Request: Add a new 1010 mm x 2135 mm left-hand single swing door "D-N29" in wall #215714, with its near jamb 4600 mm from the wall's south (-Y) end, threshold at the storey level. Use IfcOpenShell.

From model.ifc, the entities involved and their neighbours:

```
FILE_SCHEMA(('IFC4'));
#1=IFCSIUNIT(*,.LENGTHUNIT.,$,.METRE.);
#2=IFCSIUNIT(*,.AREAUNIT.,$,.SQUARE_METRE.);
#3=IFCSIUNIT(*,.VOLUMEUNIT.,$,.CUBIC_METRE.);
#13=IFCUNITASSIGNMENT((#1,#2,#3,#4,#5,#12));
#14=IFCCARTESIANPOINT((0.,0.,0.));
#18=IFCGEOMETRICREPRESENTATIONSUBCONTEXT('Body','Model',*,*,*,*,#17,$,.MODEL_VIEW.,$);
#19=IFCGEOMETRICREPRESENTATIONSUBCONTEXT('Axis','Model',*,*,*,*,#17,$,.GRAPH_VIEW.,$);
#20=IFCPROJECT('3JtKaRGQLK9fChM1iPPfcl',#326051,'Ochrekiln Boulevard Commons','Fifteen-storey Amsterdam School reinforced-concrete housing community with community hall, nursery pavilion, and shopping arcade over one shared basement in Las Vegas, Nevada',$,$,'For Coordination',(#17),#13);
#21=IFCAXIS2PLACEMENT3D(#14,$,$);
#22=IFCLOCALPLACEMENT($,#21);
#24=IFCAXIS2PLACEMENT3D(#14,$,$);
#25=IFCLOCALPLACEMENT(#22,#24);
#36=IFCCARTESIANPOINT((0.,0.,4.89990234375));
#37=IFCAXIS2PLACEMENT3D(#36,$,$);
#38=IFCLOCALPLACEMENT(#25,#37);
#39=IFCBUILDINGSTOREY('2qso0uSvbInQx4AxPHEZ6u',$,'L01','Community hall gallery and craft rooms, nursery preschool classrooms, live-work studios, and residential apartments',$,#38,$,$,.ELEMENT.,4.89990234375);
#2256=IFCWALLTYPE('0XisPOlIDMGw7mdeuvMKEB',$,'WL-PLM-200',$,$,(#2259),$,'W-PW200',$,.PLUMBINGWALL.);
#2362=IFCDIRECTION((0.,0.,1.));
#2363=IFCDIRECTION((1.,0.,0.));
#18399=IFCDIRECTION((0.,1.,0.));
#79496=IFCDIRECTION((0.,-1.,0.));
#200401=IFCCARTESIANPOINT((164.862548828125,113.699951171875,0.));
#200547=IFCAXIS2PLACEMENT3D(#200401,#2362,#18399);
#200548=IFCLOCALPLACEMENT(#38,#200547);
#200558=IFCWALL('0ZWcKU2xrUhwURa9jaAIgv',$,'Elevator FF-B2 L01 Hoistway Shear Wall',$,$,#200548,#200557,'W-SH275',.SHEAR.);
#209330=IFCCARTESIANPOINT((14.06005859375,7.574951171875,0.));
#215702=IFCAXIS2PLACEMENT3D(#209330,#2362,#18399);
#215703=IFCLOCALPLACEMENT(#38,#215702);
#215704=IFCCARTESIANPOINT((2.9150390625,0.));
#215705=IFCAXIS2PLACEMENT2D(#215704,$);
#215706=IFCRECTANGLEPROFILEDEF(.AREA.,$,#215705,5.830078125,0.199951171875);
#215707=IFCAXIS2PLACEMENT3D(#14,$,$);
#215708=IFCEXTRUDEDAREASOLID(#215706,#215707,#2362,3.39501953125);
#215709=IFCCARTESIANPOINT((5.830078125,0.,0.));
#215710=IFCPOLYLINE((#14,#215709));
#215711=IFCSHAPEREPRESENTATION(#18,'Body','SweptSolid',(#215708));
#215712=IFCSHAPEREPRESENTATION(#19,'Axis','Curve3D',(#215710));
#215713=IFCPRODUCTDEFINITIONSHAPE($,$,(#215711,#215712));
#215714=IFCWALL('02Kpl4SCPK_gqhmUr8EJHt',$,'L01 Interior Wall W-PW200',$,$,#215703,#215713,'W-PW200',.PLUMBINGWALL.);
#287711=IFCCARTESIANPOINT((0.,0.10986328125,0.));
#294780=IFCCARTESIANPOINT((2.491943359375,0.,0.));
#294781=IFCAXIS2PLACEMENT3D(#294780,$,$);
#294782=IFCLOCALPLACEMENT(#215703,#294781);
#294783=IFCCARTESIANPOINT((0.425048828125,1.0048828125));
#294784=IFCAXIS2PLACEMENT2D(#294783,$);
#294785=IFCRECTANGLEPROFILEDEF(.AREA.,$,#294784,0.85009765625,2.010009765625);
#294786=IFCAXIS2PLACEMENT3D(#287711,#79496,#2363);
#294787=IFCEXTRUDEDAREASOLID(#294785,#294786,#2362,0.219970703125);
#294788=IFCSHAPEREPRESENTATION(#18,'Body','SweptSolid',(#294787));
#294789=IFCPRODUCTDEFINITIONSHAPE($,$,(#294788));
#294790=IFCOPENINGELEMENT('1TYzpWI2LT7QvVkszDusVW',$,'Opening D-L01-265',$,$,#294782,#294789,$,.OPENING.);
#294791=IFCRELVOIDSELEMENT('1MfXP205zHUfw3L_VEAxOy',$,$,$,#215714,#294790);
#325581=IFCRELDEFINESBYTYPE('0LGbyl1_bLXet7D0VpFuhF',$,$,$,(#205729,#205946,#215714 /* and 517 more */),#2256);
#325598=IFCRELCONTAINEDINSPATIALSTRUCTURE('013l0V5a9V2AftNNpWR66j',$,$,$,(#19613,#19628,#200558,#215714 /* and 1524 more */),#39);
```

```python
import numpy as np
import ifcopenshell
import ifcopenshell.api.feature
import ifcopenshell.api.geometry
import ifcopenshell.api.root
import ifcopenshell.api.spatial
import ifcopenshell.geom
import ifcopenshell.util.element
import ifcopenshell.util.placement
import ifcopenshell.util.representation
import ifcopenshell.util.shape
import ifcopenshell.util.unit

model = ifcopenshell.open("model.ifc")
unit_scale = ifcopenshell.util.unit.calculate_unit_scale(model)
settings = ifcopenshell.geom.settings()


def volume(element):
    """Net volume in cubic metres, openings subtracted."""
    shape = ifcopenshell.geom.create_shape(settings, element)
    return ifcopenshell.util.shape.get_volume(shape.geometry)


wall = model.by_guid("02Kpl4SCPK_gqhmUr8EJHt")
storey = ifcopenshell.util.element.get_container(wall, ifc_class="IfcBuildingStorey")
context = ifcopenshell.util.representation.get_context(model, "Model", "Body", "MODEL_VIEW")
before = volume(wall)

width, height, from_end, sill = 1.01, 2.135, 4.6, 0.0  # metres

# The wall runs along its own X axis, and the end named is its -X end.
wall_shape = ifcopenshell.geom.create_shape(settings, wall)
x, y, z = ifcopenshell.util.shape.get_vertices(wall_shape.geometry).T
start = x.min() + from_end
face, thickness = float(y.min()), float(y.max() - y.min())
wall_matrix = ifcopenshell.util.placement.get_local_placement(wall.ObjectPlacement)
level = ifcopenshell.util.placement.get_local_placement(storey.ObjectPlacement)[2, 3]


def in_wall(x, y):
    """Placement at x, y metres in the wall's axes, at sill height."""
    matrix = wall_matrix.copy()
    matrix[:, 3] = wall_matrix @ np.array([x / unit_scale, y / unit_scale, 0.0, 1.0])
    matrix[2, 3] = level + sill / unit_scale
    return matrix


# Opening: a box that overshoots both wall faces by 50 mm.
opening = ifcopenshell.api.root.create_entity(model, ifc_class="IfcOpeningElement", predefined_type="OPENING")
box = ifcopenshell.api.geometry.add_wall_representation(
    model, context=context, length=width, height=height, thickness=thickness + 0.1
)
ifcopenshell.api.geometry.assign_representation(model, product=opening, representation=box)
ifcopenshell.api.geometry.edit_object_placement(model, product=opening, matrix=in_wall(start, face - 0.05), is_si=False)
ifcopenshell.api.feature.add_feature(model, feature=opening, element=wall)

door = ifcopenshell.api.root.create_entity(model, ifc_class="IfcDoor", name="D-N29", predefined_type="DOOR")
door.OverallWidth, door.OverallHeight = width / unit_scale, height / unit_scale
door.OperationType = "SINGLE_SWING_LEFT"
body = ifcopenshell.api.geometry.add_door_representation(
    model,
    context=context,
    overall_width=door.OverallWidth,
    overall_height=door.OverallHeight,
    operation_type="SINGLE_SWING_LEFT",
    lining_properties={"LiningDepth": thickness / unit_scale, "ThresholdDepth": thickness / unit_scale},
)
ifcopenshell.api.geometry.assign_representation(model, product=door, representation=body)
ifcopenshell.api.spatial.assign_container(model, products=[door], relating_structure=storey)
ifcopenshell.api.feature.add_filling(model, opening=opening, element=door)

# The lining spans the wall, so the door starts at the wall face.
ifcopenshell.api.geometry.edit_object_placement(model, product=door, matrix=in_wall(start, face), is_si=False)

after = volume(wall)

print(f"wall volume {before:.3f} -> {after:.3f} m3")

model.write("model_updated.ifc")
```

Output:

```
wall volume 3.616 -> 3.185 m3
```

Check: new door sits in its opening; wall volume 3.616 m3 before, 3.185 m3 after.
